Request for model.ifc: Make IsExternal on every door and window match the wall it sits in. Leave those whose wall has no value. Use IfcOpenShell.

First a look at what the model holds.

```python
import ifcopenshell
import ifcopenshell.util.element

model = ifcopenshell.open("model.ifc")
print(model.schema)
seen = {}
for e in model.by_type("IfcDoor") + model.by_type("IfcWindow"):
    if not e.FillsVoids:
        continue
    host = e.FillsVoids[0].RelatingOpeningElement.VoidsElements[0].RelatingBuildingElement
    own = ifcopenshell.util.element.get_pset(e, f"Pset_{e.is_a()[3:].removesuffix('StandardCase')}Common", "IsExternal")
    wall = ifcopenshell.util.element.get_pset(host, "Pset_WallCommon", "IsExternal")
    seen[e.is_a(), own, wall] = seen.get((e.is_a(), own, wall), 0) + 1
for (cls, own, wall), count in sorted(seen.items(), key=str):
    print(count, cls, "IsExternal:", own, "| host wall:", wall)
```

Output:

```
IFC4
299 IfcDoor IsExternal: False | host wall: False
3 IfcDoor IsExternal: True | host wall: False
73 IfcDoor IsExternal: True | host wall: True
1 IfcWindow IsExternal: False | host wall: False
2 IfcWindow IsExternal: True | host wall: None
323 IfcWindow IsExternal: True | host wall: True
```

```python
import ifcopenshell
import ifcopenshell.api.pset
import ifcopenshell.util.element

model = ifcopenshell.open("model.ifc")

count = 0
for ifc_class, pset_name in (("IfcDoor", "Pset_DoorCommon"), ("IfcWindow", "Pset_WindowCommon")):
    for e in model.by_type(ifc_class):
        if not e.FillsVoids:
            continue
        host = e.FillsVoids[0].RelatingOpeningElement.VoidsElements[0].RelatingBuildingElement
        external = ifcopenshell.util.element.get_pset(host, "Pset_WallCommon", "IsExternal")
        if external is None or ifcopenshell.util.element.get_pset(e, pset_name, "IsExternal") == external:
            continue
        pset = ifcopenshell.api.pset.add_pset(model, product=e, name=pset_name)
        ifcopenshell.api.pset.edit_pset(model, pset=pset, properties={"IsExternal": external})
        count += 1

print(count, "updated")

model.write("model-out.ifc")
```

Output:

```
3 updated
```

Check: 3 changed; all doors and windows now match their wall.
